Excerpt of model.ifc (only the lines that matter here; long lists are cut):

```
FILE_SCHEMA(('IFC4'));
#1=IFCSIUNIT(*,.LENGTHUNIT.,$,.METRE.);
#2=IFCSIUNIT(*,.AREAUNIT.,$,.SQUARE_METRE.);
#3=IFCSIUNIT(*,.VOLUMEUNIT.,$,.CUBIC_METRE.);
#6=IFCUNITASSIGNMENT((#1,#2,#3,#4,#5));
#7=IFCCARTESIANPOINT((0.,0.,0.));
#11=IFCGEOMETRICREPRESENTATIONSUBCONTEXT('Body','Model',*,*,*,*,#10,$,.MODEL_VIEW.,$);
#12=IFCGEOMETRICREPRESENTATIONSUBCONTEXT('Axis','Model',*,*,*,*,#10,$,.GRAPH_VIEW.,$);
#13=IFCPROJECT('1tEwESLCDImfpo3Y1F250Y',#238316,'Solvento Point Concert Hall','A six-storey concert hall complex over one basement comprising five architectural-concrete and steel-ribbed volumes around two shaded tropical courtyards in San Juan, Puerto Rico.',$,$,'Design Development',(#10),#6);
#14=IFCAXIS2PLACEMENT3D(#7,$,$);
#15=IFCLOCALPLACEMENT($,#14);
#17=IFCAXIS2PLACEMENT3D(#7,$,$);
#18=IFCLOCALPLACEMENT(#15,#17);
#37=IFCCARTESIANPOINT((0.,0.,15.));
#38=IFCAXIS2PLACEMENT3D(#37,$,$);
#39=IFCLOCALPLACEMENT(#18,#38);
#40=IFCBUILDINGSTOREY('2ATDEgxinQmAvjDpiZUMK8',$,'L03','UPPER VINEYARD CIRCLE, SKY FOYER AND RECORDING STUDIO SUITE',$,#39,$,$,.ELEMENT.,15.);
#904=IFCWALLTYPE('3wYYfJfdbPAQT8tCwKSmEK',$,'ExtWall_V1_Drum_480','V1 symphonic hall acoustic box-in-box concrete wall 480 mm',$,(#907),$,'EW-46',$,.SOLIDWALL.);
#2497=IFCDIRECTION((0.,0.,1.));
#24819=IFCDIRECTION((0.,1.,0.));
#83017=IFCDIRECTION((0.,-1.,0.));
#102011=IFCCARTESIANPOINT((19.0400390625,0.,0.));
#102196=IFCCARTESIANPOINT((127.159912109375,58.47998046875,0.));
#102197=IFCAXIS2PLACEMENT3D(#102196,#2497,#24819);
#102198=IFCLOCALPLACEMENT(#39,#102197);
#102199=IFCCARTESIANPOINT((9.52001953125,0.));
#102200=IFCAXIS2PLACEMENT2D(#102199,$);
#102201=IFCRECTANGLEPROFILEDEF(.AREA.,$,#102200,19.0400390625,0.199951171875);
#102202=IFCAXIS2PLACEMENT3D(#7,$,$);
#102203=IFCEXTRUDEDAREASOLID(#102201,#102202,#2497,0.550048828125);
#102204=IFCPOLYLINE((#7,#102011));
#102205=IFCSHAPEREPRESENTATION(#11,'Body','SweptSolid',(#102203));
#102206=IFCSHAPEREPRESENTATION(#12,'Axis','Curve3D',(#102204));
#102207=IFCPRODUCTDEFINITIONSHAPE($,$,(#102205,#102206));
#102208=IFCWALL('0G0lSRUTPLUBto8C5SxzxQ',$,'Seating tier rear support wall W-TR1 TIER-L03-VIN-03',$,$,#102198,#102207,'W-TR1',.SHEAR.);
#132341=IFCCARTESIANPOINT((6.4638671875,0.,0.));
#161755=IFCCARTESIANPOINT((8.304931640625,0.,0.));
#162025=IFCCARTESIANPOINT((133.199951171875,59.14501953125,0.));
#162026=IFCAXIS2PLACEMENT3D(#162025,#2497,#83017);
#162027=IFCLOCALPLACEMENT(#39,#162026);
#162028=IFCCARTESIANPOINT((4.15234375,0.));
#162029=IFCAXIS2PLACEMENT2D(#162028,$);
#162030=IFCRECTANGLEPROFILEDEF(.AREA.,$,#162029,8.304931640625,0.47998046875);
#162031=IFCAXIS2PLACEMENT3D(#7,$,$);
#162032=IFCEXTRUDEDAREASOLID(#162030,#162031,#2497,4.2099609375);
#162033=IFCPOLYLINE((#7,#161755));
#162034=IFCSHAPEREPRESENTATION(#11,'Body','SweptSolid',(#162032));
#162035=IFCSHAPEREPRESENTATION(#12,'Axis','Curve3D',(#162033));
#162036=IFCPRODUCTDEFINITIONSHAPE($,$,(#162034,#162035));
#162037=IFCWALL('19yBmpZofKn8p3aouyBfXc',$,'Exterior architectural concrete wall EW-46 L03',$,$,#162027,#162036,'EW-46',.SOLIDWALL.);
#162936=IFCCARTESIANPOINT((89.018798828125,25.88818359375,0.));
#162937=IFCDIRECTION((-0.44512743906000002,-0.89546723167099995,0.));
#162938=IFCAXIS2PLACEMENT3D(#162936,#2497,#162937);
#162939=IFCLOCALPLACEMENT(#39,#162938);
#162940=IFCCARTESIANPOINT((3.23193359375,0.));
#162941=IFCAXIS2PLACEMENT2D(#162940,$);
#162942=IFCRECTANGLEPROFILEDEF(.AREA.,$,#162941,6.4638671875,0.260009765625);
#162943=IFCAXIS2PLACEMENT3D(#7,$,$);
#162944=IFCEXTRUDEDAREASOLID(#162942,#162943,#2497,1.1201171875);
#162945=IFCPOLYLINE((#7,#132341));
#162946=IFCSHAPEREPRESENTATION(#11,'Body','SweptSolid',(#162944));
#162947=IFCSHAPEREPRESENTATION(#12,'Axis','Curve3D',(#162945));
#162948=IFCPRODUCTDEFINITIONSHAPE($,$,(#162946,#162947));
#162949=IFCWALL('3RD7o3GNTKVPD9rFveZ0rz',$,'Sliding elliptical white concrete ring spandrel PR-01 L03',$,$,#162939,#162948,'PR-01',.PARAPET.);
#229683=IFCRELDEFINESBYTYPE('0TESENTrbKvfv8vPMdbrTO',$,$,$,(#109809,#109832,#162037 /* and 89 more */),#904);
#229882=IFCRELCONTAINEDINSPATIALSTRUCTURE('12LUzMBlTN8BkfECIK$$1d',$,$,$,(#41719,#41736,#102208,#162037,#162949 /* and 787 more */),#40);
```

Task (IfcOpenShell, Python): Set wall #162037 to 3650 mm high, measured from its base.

```python
import ifcopenshell
import ifcopenshell.geom
import ifcopenshell.util.representation
import ifcopenshell.util.shape
import ifcopenshell.util.unit

model = ifcopenshell.open("model.ifc")
unit_scale = ifcopenshell.util.unit.calculate_unit_scale(model)
settings = ifcopenshell.geom.settings()


def volume(element):
    """Net volume in cubic metres, openings subtracted."""
    shape = ifcopenshell.geom.create_shape(settings, element)
    return ifcopenshell.util.shape.get_volume(shape.geometry)


wall = model.by_id(162037)
before = volume(wall)

body = ifcopenshell.util.representation.get_representation(wall, "Model", "Body")
solid = body.Items[0]
old_height = solid.Depth
solid.Depth = 3.65 / unit_scale
after = volume(wall)

print(f"height {old_height:g} -> {solid.Depth:g}, volume {before:.3f} -> {after:.3f} m3")

model.write("model_edited.ifc")
```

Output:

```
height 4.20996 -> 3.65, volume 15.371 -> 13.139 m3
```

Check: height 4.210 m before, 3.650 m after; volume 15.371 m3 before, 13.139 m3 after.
